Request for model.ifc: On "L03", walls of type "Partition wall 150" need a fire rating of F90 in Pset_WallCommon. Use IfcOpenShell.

First a look at what the model holds.

```python
import ifcopenshell
import ifcopenshell.util.element

model = ifcopenshell.open("model.ifc")
print(model.schema)
storey = next(s for s in model.by_type("IfcBuildingStorey") if s.Name == "L03")
walls = [e for e in ifcopenshell.util.element.get_decomposition(storey) if e.is_a("IfcWall")]
seen = {}
for e in walls:
    element_type = ifcopenshell.util.element.get_type(e)
    key = (element_type.Name if element_type != e and element_type else None, ifcopenshell.util.element.get_pset(e, "Pset_WallCommon", "FireRating"))
    seen[key] = seen.get(key, 0) + 1
for (name, value), count in sorted(seen.items(), key=str):
    print(count, "x", name, "|", value)
```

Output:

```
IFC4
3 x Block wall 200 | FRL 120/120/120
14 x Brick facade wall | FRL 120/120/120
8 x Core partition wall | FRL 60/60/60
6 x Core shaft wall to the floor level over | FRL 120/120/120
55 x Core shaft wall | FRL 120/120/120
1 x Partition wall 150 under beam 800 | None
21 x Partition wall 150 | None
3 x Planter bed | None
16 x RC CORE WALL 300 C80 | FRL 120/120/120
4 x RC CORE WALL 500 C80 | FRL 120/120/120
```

```python
import ifcopenshell
import ifcopenshell.api.pset
import ifcopenshell.util.element

model = ifcopenshell.open("model.ifc")

storey = next(s for s in model.by_type("IfcBuildingStorey") if s.Name == "L03")
walls = [e for e in ifcopenshell.util.element.get_decomposition(storey) if e.is_a("IfcWall")]

count = 0
for e in walls:
    element_type = ifcopenshell.util.element.get_type(e)
    if element_type in (None, e) or element_type.Name != "Partition wall 150":
        continue
    found = ifcopenshell.util.element.get_pset(e, "Pset_WallCommon", should_inherit=False)
    if found:
        pset = model.by_id(found["id"])
        if len(ifcopenshell.util.element.get_elements_by_pset(pset)) > 1:
            pset = ifcopenshell.api.pset.unshare_pset(model, products=[e], pset=pset)[0]
    else:
        pset = ifcopenshell.api.pset.add_pset(model, product=e, name="Pset_WallCommon")
    ifcopenshell.api.pset.edit_pset(model, pset=pset, properties={"FireRating": "F90"})
    count += 1

print(count, "walls updated")

model.write("model-out.ifc")
```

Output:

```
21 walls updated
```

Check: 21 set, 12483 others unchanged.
